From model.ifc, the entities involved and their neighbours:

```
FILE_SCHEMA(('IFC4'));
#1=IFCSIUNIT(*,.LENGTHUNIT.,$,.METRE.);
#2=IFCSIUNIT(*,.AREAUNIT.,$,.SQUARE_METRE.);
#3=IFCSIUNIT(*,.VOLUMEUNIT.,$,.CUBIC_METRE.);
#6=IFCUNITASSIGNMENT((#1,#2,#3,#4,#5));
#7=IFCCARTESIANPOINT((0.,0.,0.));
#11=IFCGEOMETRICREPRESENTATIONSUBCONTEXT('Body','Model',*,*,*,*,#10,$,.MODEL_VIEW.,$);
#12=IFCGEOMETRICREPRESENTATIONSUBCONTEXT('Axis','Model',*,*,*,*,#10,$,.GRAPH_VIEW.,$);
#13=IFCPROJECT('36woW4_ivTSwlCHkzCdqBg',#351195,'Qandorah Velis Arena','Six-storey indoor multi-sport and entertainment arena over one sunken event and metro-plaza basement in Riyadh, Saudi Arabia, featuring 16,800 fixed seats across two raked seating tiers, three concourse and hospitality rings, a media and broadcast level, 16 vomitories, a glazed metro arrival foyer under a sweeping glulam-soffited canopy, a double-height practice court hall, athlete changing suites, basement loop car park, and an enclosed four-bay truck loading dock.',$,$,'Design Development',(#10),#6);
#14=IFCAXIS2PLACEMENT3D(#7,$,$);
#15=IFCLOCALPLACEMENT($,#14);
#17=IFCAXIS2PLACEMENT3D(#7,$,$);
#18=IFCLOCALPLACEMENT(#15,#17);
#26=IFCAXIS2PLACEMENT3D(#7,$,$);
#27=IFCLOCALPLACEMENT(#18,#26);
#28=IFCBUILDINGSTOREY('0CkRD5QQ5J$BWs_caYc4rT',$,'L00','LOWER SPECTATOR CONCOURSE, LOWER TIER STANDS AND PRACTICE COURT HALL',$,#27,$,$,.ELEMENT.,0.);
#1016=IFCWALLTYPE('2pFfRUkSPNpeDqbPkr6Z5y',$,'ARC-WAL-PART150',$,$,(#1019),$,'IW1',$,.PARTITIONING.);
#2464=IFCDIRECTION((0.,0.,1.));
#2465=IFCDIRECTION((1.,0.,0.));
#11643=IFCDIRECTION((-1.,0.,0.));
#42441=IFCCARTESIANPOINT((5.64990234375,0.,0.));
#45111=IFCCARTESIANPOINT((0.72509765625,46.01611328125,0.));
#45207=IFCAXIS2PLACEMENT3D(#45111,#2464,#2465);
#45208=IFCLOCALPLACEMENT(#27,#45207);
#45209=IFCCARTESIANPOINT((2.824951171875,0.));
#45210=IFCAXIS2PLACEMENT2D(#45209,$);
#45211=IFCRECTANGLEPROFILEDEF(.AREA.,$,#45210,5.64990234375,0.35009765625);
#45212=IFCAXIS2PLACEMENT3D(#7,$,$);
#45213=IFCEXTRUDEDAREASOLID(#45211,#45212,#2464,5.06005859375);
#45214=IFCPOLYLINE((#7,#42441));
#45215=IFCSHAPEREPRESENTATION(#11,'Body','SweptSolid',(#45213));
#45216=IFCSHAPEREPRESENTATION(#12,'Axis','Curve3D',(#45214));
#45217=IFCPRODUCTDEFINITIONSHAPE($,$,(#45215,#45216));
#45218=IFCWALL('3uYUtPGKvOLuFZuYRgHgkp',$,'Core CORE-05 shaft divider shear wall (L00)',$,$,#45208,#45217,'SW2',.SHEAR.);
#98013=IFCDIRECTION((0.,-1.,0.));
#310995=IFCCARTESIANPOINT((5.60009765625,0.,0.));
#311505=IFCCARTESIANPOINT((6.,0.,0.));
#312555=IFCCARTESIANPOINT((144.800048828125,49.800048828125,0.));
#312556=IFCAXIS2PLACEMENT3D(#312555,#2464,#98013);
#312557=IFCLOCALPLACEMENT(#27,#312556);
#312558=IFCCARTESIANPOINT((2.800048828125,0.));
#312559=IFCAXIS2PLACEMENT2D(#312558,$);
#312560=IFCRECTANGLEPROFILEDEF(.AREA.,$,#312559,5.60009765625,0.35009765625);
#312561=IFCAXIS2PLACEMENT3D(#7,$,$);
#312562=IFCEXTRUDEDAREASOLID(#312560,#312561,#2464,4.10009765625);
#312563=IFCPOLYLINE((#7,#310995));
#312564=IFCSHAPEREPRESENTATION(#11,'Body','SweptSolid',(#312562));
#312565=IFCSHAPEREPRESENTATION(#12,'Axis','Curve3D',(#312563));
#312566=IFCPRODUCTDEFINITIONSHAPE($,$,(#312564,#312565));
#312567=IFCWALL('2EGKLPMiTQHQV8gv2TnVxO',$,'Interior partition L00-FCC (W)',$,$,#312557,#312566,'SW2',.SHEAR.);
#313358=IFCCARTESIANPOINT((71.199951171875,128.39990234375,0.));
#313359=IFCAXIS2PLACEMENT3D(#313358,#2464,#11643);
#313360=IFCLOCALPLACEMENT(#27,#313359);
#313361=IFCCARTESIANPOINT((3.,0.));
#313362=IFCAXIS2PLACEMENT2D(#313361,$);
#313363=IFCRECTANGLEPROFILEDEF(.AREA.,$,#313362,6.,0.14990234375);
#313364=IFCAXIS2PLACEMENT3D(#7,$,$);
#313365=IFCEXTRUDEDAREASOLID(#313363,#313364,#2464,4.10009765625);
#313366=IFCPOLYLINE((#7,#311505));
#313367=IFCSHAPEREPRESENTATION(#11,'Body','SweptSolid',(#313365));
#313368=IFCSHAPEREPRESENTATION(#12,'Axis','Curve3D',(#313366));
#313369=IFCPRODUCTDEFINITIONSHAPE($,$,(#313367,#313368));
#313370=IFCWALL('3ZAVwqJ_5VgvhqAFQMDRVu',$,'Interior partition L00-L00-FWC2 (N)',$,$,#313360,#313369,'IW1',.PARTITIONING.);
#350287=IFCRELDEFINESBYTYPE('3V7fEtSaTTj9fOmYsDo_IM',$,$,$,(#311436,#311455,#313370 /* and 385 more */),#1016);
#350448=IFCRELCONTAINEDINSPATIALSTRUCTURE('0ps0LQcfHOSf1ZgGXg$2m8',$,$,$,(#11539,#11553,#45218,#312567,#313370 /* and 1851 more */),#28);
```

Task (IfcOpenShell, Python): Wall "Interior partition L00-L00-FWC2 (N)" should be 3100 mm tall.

```python
import ifcopenshell
import ifcopenshell.geom
import ifcopenshell.util.representation
import ifcopenshell.util.shape

model = ifcopenshell.open("model.ifc")
settings = ifcopenshell.geom.settings()


def volume(element):
    """Net volume in cubic metres, openings subtracted."""
    shape = ifcopenshell.geom.create_shape(settings, element)
    return ifcopenshell.util.shape.get_volume(shape.geometry)


wall = model.by_guid("3ZAVwqJ_5VgvhqAFQMDRVu")
before = volume(wall)

body = ifcopenshell.util.representation.get_representation(wall, "Model", "Body")
solid = body.Items[0]
old_height = solid.Depth
solid.Depth = 3.1
after = volume(wall)

print(f"height {old_height:g} -> {solid.Depth:g}, volume {before:.3f} -> {after:.3f} m3")

model.write("model_rev.ifc")
```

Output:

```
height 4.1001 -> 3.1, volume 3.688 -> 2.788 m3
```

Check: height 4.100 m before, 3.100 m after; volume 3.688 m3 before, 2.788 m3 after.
